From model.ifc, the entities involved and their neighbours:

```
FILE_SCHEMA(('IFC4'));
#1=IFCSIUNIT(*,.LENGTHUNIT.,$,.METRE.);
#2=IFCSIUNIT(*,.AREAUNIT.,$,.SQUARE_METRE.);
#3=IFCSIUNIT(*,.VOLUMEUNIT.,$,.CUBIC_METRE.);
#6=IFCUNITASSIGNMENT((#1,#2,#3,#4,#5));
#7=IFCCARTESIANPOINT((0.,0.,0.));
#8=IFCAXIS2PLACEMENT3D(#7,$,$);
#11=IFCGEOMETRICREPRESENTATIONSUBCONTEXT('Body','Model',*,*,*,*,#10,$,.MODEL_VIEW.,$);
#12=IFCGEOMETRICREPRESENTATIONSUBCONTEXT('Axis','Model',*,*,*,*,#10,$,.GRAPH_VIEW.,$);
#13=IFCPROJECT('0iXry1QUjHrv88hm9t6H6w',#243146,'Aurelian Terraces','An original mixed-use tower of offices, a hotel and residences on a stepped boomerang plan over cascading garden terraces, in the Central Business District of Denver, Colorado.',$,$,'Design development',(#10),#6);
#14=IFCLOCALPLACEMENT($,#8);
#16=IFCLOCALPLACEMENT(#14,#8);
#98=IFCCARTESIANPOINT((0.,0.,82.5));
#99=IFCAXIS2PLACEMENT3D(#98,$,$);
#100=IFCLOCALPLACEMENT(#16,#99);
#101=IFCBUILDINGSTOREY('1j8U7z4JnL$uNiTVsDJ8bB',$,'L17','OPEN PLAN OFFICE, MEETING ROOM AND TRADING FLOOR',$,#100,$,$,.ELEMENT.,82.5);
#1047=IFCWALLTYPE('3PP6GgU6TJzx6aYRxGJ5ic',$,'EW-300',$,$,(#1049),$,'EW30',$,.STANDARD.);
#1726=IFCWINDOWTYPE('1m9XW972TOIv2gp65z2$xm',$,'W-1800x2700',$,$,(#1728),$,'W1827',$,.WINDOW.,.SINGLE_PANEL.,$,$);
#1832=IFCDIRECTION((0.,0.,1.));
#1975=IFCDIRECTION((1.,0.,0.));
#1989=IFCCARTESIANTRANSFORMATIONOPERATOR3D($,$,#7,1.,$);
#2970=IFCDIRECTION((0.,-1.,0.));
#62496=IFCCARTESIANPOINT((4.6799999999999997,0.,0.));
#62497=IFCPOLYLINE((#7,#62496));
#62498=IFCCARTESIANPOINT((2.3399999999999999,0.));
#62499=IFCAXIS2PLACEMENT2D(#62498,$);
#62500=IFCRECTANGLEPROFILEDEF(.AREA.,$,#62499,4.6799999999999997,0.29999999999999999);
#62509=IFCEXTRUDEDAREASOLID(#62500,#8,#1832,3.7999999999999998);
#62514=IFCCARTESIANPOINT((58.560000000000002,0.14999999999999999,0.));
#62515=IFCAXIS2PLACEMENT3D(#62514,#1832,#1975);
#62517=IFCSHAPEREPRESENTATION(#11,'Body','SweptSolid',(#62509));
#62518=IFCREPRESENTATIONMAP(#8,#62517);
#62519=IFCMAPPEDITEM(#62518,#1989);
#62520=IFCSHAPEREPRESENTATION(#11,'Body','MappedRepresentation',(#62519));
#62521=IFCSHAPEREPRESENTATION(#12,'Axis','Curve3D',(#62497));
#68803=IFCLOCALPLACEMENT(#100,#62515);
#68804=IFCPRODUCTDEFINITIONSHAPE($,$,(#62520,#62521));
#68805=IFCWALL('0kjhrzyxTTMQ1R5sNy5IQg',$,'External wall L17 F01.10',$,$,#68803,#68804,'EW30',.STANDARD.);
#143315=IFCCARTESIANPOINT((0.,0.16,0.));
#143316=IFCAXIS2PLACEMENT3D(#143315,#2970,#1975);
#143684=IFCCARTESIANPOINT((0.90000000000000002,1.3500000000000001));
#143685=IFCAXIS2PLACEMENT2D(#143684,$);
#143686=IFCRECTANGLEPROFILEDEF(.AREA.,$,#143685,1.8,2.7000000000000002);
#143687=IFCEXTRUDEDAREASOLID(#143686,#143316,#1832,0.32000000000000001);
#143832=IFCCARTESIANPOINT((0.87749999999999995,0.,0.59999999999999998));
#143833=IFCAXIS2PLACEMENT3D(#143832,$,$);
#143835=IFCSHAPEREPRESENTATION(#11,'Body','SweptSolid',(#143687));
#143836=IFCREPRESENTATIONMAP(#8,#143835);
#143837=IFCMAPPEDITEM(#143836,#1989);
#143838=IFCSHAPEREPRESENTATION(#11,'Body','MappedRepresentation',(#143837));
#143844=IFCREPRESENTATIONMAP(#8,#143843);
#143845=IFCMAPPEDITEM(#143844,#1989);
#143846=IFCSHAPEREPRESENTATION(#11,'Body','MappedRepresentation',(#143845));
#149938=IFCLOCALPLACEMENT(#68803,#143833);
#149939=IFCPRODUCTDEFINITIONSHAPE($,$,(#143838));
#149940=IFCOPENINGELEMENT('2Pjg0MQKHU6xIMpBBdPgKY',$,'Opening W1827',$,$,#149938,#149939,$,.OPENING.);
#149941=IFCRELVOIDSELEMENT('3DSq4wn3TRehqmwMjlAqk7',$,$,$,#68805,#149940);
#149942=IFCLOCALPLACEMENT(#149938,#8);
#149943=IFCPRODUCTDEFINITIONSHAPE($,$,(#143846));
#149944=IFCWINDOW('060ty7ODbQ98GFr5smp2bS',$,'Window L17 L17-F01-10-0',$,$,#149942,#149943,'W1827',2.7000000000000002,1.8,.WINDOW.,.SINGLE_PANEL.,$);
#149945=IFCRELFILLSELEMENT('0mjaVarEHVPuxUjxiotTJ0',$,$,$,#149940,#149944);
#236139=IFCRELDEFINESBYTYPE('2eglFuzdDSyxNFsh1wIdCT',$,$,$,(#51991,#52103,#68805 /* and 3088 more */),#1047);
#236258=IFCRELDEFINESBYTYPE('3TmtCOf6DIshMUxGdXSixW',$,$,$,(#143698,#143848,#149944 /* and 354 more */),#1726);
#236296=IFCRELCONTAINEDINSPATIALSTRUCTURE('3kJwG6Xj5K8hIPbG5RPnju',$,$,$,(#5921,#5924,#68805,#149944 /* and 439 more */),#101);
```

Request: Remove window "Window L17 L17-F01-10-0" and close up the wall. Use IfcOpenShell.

```python
import ifcopenshell
import ifcopenshell.api.feature
import ifcopenshell.api.root
import ifcopenshell.geom
import ifcopenshell.util.shape

model = ifcopenshell.open("model.ifc")
settings = ifcopenshell.geom.settings()


def volume(element):
    """Net volume in cubic metres, openings subtracted."""
    shape = ifcopenshell.geom.create_shape(settings, element)
    return ifcopenshell.util.shape.get_volume(shape.geometry)


window = model.by_id(149944)
opening = window.FillsVoids[0].RelatingOpeningElement
wall = opening.VoidsElements[0].RelatingBuildingElement
before = volume(wall)

ifcopenshell.api.root.remove_product(model, product=window)
ifcopenshell.api.feature.remove_feature(model, feature=opening)

after = volume(wall)

print(f"wall volume {before:.3f} -> {after:.3f} m3")

model.write("model_v2.ifc")
```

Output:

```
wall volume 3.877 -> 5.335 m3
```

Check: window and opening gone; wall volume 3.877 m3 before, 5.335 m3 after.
